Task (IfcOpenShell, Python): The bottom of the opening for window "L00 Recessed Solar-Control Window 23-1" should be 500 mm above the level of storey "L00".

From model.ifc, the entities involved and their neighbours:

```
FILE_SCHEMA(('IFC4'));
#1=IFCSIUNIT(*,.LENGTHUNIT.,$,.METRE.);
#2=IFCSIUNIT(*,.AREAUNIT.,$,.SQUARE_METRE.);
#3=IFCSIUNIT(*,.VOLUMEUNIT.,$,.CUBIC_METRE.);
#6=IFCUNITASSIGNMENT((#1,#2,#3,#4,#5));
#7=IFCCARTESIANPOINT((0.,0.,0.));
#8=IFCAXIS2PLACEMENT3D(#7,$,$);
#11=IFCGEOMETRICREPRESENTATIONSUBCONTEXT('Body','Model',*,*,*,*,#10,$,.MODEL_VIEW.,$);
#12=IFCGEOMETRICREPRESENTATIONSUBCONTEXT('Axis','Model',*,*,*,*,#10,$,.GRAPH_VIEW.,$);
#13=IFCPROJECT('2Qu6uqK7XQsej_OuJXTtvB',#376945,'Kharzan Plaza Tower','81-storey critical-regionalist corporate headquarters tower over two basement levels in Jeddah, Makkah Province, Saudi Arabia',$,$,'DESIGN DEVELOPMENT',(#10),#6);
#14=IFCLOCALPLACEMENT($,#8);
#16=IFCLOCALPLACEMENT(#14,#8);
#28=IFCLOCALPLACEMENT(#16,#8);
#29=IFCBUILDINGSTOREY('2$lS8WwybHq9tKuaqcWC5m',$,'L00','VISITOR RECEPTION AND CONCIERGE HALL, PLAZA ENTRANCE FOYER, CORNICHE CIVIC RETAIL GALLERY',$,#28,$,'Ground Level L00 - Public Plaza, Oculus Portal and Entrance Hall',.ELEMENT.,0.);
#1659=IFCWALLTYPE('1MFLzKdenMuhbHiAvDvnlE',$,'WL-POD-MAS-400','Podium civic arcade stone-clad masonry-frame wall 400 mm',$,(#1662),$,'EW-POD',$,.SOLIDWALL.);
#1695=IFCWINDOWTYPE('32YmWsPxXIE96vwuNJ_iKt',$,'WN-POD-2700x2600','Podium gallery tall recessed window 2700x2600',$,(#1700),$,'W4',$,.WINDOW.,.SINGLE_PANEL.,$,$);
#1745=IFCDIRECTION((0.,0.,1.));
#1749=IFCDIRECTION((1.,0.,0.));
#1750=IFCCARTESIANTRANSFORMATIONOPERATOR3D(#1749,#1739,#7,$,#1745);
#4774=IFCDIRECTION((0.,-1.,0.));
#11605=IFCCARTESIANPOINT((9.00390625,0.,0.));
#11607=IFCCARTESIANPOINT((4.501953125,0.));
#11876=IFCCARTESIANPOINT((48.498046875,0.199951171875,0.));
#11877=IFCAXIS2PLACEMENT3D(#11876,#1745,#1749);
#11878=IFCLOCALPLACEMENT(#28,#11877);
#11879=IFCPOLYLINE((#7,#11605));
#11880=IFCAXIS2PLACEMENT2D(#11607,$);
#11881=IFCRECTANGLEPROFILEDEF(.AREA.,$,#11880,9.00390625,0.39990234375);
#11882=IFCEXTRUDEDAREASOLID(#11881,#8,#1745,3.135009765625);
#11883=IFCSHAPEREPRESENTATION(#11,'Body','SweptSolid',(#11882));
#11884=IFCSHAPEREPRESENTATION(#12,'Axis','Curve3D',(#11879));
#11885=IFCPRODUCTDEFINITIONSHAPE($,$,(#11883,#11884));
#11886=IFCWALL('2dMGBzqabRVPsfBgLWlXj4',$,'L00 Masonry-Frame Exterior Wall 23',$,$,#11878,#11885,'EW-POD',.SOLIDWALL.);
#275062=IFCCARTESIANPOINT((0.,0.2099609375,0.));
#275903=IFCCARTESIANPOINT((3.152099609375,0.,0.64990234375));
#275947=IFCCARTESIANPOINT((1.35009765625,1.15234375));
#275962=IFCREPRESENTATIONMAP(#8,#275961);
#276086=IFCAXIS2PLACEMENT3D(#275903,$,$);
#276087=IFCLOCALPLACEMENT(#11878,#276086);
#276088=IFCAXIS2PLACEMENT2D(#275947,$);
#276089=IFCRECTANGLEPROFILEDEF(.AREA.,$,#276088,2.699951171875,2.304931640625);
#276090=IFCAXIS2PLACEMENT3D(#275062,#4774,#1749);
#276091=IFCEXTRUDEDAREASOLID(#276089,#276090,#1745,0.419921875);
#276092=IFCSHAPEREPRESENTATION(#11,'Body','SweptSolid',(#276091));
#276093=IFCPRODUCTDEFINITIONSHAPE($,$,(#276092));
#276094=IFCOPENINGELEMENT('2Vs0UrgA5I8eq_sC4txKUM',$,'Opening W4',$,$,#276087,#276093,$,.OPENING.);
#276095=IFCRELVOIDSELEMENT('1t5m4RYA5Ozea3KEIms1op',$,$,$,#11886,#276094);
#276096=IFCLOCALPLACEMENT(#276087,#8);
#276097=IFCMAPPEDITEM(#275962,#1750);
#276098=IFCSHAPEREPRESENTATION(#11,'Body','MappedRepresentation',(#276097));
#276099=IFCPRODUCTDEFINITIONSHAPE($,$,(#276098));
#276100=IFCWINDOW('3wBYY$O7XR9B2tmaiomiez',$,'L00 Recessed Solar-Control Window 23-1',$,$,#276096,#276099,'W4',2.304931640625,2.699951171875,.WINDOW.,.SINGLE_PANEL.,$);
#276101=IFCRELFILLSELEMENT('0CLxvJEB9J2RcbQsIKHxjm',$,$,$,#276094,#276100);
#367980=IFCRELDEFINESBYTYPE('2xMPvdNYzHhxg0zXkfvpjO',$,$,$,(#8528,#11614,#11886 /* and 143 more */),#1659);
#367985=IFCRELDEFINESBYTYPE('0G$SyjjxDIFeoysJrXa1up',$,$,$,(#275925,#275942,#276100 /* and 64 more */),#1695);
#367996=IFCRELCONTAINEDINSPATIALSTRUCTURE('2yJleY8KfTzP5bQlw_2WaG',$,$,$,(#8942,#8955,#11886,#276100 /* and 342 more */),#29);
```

```python
import numpy as np
import ifcopenshell
import ifcopenshell.api.geometry
import ifcopenshell.geom
import ifcopenshell.util.element
import ifcopenshell.util.placement
import ifcopenshell.util.shape
import ifcopenshell.util.unit

model = ifcopenshell.open("model.ifc")
unit_scale = ifcopenshell.util.unit.calculate_unit_scale(model)

window = model.by_id(276100)
opening = window.FillsVoids[0].RelatingOpeningElement
storey = ifcopenshell.util.element.get_container(window, ifc_class="IfcBuildingStorey")
level = ifcopenshell.util.placement.get_local_placement(storey.ObjectPlacement)[2, 3]

# The opening's origin need not be at the sill, so measure its lowest point.
shape = ifcopenshell.geom.create_shape(ifcopenshell.geom.settings(), opening)
bottom = ifcopenshell.util.shape.get_shape_bottom_elevation(shape, shape.geometry) / unit_scale
dz = level + 0.5 / unit_scale - bottom

shift = np.array([0.0, 0.0, dz])
# The window is placed relative to its opening, so it follows when the opening moves.
matrix = ifcopenshell.util.placement.get_local_placement(opening.ObjectPlacement)
matrix[:3, 3] += shift
ifcopenshell.api.geometry.edit_object_placement(
    model, product=opening, matrix=matrix, is_si=False, should_transform_children=True
)

print(f"moved by {dz * unit_scale:+.3f} m")

model.write("model_edited.ifc")
```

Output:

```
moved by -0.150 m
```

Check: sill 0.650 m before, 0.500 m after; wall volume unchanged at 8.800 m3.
